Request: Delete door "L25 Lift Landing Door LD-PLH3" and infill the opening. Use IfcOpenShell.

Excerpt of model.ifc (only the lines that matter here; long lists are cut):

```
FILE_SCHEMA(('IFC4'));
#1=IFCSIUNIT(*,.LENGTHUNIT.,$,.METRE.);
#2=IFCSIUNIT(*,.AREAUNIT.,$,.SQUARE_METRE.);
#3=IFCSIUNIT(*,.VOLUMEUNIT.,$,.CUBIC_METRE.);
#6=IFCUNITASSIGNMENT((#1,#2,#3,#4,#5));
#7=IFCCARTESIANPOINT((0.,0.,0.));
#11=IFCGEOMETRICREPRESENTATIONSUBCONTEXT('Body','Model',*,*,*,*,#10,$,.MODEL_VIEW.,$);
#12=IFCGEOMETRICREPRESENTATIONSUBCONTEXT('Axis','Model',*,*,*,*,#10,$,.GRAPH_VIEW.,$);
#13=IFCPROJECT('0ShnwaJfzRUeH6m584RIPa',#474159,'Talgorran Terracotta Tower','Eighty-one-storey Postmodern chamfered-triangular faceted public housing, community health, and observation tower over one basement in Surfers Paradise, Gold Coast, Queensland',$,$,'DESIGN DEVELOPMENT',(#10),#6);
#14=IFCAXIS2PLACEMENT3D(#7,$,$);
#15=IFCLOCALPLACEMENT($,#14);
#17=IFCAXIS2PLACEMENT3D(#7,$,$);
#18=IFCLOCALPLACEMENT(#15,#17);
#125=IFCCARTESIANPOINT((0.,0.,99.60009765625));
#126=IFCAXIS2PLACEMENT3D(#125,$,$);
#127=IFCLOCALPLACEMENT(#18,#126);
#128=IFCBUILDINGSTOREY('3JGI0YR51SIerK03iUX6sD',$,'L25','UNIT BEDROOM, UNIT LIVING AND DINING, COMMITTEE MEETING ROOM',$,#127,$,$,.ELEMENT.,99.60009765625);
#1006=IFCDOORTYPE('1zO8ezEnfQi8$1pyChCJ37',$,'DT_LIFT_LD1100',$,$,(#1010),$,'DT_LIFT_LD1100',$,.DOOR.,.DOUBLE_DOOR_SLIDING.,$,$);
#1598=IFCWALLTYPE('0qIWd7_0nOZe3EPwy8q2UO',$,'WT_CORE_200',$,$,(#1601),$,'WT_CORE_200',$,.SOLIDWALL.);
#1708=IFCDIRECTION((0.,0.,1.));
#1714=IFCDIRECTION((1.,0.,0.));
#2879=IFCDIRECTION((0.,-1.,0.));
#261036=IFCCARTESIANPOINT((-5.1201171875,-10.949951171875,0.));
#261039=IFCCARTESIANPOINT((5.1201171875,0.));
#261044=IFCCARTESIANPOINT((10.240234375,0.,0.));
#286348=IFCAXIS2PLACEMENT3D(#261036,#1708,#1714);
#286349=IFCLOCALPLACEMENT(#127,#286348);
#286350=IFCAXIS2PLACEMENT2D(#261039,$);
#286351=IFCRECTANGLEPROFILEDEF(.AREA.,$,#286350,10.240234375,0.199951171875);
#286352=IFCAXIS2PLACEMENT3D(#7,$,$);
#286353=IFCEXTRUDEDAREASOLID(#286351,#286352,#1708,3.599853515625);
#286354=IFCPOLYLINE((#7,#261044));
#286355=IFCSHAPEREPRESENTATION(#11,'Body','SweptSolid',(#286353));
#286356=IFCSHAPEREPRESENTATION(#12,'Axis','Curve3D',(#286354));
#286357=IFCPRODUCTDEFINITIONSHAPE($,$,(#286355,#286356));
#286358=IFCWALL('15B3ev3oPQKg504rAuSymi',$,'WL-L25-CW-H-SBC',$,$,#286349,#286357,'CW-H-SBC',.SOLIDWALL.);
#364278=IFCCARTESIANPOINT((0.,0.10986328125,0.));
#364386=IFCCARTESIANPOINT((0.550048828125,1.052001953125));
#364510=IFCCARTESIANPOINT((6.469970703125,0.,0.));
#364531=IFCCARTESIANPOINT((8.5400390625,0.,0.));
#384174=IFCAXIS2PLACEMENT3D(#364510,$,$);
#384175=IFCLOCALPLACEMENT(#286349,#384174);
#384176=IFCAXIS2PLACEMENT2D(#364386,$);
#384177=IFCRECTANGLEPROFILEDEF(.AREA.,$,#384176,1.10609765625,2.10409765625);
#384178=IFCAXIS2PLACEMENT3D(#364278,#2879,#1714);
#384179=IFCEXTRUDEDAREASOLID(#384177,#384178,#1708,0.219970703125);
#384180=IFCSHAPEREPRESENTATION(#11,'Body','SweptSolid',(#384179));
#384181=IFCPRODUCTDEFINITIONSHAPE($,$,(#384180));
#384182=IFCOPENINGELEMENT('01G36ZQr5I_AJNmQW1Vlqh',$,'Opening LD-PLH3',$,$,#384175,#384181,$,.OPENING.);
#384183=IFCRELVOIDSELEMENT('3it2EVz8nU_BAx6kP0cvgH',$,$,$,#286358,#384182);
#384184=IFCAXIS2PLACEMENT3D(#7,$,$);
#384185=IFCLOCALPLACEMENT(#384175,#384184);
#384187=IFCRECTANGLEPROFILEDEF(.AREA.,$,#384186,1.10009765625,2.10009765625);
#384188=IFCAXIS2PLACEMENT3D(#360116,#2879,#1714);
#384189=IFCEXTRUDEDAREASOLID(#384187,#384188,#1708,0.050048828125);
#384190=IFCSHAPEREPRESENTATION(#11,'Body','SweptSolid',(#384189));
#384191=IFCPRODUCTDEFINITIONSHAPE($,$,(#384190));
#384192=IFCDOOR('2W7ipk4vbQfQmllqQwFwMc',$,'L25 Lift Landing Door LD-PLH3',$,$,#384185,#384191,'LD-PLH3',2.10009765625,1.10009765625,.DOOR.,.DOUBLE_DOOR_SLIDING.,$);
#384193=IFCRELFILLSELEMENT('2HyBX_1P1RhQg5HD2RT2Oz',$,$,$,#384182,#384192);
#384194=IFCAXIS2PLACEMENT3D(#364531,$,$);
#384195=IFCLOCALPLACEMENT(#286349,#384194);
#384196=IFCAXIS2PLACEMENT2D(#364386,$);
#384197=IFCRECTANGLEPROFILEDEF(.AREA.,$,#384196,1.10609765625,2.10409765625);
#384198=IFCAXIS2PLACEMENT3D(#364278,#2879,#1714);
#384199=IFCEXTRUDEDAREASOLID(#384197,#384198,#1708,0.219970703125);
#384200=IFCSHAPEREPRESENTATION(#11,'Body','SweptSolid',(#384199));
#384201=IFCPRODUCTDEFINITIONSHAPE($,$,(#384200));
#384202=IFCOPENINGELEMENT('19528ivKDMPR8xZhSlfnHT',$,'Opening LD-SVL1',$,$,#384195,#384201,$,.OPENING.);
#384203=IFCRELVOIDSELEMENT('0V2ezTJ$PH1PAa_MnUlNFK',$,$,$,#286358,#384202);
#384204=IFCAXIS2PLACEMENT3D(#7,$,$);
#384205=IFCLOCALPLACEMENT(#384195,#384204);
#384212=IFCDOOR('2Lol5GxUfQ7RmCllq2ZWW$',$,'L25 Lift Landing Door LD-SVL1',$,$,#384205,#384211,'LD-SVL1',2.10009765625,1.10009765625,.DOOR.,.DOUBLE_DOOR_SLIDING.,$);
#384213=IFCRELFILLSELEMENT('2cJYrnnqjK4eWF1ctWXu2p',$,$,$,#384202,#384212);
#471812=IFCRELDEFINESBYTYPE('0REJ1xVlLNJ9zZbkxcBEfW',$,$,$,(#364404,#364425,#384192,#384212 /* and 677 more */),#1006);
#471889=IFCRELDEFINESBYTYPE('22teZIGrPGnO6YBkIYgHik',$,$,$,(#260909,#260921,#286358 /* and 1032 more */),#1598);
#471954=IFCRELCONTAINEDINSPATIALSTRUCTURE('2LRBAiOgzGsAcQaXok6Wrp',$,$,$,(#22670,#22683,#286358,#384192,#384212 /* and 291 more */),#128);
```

```python
import ifcopenshell
import ifcopenshell.api.feature
import ifcopenshell.api.root
import ifcopenshell.geom
import ifcopenshell.util.shape

model = ifcopenshell.open("model.ifc")
settings = ifcopenshell.geom.settings()


def volume(element):
    """Net volume in cubic metres, openings subtracted."""
    shape = ifcopenshell.geom.create_shape(settings, element)
    return ifcopenshell.util.shape.get_volume(shape.geometry)


door = model.by_guid("2W7ipk4vbQfQmllqQwFwMc")
opening = door.FillsVoids[0].RelatingOpeningElement
wall = opening.VoidsElements[0].RelatingBuildingElement
before = volume(wall)

ifcopenshell.api.root.remove_product(model, product=door)
ifcopenshell.api.feature.remove_feature(model, feature=opening)

after = volume(wall)

print(f"wall volume {before:.3f} -> {after:.3f} m3")

model.write("model_rev.ifc")
```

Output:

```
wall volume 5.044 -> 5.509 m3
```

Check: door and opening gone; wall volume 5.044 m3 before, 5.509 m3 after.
